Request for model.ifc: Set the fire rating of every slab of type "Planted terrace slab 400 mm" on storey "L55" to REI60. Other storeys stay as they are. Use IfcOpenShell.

First a look at what the model holds.

```python
import ifcopenshell
import ifcopenshell.util.element

model = ifcopenshell.open("model.ifc")
print(model.schema)
storey = next(s for s in model.by_type("IfcBuildingStorey") if s.Name == "L55")
slabs = [e for e in ifcopenshell.util.element.get_decomposition(storey) if e.is_a("IfcSlab")]
seen = {}
for e in slabs:
    element_type = ifcopenshell.util.element.get_type(e)
    key = (element_type.Name if element_type != e and element_type else None, ifcopenshell.util.element.get_pset(e, "Pset_SlabCommon", "FireRating"))
    seen[key] = seen.get(key, 0) + 1
for (name, value), count in sorted(seen.items(), key=str):
    print(count, "x", name, "|", value)
```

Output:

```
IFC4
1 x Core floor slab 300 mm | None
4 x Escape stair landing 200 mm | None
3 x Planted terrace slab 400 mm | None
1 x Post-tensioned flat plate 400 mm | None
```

```python
import ifcopenshell
import ifcopenshell.api.pset
import ifcopenshell.util.element

model = ifcopenshell.open("model.ifc")

storey = next(s for s in model.by_type("IfcBuildingStorey") if s.Name == "L55")
slabs = [e for e in ifcopenshell.util.element.get_decomposition(storey) if e.is_a("IfcSlab")]

count = 0
for e in slabs:
    element_type = ifcopenshell.util.element.get_type(e)
    if element_type in (None, e) or element_type.Name != "Planted terrace slab 400 mm":
        continue
    found = ifcopenshell.util.element.get_pset(e, "Pset_SlabCommon", should_inherit=False)
    if found:
        pset = model.by_id(found["id"])
        if len(ifcopenshell.util.element.get_elements_by_pset(pset)) > 1:
            pset = ifcopenshell.api.pset.unshare_pset(model, products=[e], pset=pset)[0]
    else:
        pset = ifcopenshell.api.pset.add_pset(model, product=e, name="Pset_SlabCommon")
    ifcopenshell.api.pset.edit_pset(model, pset=pset, properties={"FireRating": "REI60"})
    count += 1

print(count, "slabs updated")

model.write("model-out.ifc")
```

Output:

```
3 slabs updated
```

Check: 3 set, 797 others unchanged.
